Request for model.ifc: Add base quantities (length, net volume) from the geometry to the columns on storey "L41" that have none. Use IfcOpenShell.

First a look at what the model holds.

```python
import ifcopenshell
import ifcopenshell.util.element
import ifcopenshell.util.unit

model = ifcopenshell.open("model.ifc")
print(model.schema)
for unit_type in ("LENGTHUNIT", "AREAUNIT", "VOLUMEUNIT"):
    print(unit_type, ifcopenshell.util.unit.calculate_unit_scale(model, unit_type))
storey = next(s for s in model.by_type("IfcBuildingStorey") if s.Name == "L41")
columns = [e for e in ifcopenshell.util.element.get_decomposition(storey) if e.is_a("IfcColumn")]
for e in sorted(columns, key=lambda e: e.id()):
    print(e.id(), e.is_a(), e.Name, list(ifcopenshell.util.element.get_psets(e, qtos_only=True)), sep=" | ")
```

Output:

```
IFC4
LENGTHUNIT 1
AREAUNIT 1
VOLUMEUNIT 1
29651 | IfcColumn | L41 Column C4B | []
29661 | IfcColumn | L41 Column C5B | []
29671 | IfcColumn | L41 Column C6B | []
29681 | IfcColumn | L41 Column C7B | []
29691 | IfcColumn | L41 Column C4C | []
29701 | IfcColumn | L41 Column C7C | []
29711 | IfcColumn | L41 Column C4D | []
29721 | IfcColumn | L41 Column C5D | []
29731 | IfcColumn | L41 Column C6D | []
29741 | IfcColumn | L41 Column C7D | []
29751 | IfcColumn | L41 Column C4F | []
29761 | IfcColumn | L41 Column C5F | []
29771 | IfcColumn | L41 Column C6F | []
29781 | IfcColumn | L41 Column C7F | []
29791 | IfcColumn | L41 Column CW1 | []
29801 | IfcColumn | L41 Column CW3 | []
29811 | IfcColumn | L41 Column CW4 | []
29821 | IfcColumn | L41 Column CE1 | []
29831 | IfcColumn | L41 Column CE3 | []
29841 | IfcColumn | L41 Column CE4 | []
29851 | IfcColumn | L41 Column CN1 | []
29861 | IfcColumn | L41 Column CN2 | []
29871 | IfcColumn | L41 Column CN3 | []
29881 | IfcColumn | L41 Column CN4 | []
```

```python
import ifcopenshell
import ifcopenshell.api.pset
import ifcopenshell.geom
import ifcopenshell.util.element
import ifcopenshell.util.shape
import ifcopenshell.util.unit

model = ifcopenshell.open("model.ifc")
unit_scale = ifcopenshell.util.unit.calculate_unit_scale(model)
volume_scale = ifcopenshell.util.unit.calculate_unit_scale(model, "VOLUMEUNIT")
settings = ifcopenshell.geom.settings()

storey = next(s for s in model.by_type("IfcBuildingStorey") if s.Name == "L41")
columns = [e for e in ifcopenshell.util.element.get_decomposition(storey) if e.is_a("IfcColumn")]

for e in sorted(columns, key=lambda e: e.id()):
    if ifcopenshell.util.element.get_psets(e, qtos_only=True, should_inherit=False):
        continue
    # Geometry comes back in metres, in the element's own axes.
    shape = ifcopenshell.geom.create_shape(settings, e)
    values = {
        "Length": ifcopenshell.util.shape.get_z(shape.geometry) / unit_scale,
        "NetVolume": ifcopenshell.util.shape.get_volume(shape.geometry) / volume_scale,
    }
    qto = ifcopenshell.api.pset.add_qto(model, product=e, name="Qto_ColumnBaseQuantities")
    ifcopenshell.api.pset.edit_qto(model, qto=qto, properties=values)
    print(e.id(), {k: round(v, 3) for k, v in values.items()})

model.write("model_v2.ifc")
```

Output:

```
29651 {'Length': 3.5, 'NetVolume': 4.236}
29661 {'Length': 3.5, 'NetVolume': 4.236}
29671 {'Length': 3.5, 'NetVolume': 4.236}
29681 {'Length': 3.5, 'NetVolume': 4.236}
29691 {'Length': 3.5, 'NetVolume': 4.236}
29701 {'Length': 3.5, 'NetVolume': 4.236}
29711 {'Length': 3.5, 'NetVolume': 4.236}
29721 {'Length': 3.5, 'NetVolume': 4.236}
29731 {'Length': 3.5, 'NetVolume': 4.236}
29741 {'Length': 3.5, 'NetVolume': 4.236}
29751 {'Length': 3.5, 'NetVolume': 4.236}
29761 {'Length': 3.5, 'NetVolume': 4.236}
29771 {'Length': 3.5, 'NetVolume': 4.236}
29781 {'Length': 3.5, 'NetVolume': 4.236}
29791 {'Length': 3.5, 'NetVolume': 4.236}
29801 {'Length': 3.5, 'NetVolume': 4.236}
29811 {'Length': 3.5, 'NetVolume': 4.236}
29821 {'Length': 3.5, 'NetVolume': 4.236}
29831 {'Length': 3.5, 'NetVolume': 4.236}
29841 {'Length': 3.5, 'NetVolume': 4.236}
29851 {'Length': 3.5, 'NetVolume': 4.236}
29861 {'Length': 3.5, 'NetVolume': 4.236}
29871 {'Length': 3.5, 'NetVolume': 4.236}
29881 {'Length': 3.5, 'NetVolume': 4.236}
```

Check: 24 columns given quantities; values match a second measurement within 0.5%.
